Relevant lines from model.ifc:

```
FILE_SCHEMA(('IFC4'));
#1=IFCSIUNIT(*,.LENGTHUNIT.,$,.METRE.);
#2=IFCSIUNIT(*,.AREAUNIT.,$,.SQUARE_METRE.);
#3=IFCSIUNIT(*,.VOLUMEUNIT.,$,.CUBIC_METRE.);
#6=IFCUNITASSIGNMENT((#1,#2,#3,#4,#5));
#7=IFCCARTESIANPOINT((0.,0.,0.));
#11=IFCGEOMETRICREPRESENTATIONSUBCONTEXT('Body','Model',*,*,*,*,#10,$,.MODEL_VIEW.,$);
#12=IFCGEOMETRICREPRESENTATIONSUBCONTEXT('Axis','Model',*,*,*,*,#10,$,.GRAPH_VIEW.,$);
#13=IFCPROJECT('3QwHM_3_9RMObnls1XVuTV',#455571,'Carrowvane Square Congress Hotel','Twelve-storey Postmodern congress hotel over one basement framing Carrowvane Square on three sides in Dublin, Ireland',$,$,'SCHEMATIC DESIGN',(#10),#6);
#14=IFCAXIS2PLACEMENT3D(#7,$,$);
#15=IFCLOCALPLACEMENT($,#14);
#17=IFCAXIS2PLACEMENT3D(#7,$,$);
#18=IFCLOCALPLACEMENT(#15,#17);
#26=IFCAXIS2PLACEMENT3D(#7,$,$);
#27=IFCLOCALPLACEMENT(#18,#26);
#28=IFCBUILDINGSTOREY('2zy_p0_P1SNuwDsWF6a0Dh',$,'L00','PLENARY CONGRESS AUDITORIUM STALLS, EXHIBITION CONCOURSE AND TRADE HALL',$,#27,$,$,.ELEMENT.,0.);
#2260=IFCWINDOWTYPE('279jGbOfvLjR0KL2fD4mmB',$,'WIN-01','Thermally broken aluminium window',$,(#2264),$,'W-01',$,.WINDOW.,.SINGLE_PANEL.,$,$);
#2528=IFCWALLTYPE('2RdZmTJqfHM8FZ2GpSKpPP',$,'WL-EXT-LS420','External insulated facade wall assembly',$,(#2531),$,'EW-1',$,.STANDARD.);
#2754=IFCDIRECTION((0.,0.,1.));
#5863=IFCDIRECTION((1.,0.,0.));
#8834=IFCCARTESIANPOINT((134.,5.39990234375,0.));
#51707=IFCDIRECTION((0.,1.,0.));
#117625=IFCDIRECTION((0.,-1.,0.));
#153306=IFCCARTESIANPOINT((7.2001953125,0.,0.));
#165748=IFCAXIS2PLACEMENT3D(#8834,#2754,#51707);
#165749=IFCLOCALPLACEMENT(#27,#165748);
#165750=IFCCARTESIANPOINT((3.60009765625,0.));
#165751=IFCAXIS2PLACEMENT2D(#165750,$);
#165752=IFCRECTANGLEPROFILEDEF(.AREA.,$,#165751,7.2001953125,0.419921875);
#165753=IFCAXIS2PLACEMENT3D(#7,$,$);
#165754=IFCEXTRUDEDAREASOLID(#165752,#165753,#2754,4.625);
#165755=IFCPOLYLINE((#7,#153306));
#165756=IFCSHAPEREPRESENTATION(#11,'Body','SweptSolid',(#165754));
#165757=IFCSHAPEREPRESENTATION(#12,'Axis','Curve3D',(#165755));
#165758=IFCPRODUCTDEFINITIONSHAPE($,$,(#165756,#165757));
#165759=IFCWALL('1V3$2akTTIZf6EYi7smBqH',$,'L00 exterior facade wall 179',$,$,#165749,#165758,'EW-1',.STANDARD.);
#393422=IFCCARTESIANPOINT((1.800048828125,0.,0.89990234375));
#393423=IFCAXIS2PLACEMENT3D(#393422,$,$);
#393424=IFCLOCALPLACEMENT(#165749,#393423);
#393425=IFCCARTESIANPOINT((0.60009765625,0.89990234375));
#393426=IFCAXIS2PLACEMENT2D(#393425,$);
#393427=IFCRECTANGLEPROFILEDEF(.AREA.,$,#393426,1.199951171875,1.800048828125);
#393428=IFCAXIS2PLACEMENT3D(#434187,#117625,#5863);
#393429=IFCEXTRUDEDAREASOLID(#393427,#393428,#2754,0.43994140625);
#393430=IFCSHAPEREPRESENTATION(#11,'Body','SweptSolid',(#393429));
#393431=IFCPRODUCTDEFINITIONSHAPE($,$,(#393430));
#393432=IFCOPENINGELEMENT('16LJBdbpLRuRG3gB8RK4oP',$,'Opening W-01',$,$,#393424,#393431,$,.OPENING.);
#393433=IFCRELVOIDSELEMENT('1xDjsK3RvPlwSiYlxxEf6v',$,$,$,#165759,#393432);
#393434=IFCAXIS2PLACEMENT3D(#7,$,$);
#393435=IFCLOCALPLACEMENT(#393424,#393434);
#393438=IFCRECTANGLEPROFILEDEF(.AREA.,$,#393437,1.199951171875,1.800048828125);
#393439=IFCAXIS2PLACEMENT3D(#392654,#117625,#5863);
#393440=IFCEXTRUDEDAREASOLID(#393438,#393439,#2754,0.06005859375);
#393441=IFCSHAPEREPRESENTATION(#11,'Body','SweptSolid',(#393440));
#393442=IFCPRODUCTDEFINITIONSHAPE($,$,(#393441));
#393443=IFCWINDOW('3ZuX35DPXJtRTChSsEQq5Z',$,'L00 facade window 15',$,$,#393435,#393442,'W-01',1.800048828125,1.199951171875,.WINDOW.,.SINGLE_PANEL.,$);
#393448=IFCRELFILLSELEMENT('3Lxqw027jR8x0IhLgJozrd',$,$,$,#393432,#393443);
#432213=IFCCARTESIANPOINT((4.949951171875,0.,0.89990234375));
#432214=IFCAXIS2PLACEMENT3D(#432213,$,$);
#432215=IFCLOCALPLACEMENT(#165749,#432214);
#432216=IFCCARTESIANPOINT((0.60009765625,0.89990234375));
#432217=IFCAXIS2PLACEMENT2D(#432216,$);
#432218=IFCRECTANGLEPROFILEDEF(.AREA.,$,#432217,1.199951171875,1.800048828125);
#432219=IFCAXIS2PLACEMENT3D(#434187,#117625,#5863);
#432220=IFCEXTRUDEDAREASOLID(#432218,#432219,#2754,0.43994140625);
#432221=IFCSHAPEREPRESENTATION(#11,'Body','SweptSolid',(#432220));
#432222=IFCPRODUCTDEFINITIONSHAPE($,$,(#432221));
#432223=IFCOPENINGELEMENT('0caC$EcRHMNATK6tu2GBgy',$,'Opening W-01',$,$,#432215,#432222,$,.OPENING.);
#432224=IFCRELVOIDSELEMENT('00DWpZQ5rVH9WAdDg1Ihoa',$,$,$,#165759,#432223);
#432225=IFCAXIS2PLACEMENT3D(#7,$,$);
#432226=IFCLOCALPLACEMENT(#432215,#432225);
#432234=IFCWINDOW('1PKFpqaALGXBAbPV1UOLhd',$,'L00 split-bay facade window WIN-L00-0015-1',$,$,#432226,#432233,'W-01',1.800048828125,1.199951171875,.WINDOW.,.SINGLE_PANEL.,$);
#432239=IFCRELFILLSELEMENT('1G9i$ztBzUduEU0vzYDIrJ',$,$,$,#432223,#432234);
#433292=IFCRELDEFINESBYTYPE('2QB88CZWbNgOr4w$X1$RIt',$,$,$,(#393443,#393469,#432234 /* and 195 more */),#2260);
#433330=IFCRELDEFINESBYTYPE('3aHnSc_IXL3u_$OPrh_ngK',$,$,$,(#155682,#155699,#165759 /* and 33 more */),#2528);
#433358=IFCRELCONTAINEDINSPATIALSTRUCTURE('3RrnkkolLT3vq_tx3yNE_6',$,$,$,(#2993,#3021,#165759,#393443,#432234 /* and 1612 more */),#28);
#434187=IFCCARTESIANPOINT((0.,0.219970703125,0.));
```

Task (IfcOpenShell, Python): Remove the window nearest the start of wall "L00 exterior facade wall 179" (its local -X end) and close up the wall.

```python
import ifcopenshell
import ifcopenshell.api.feature
import ifcopenshell.api.root
import ifcopenshell.geom
import ifcopenshell.util.shape

model = ifcopenshell.open("model.ifc")
settings = ifcopenshell.geom.settings()


def volume(element):
    """Net volume in cubic metres, openings subtracted."""
    shape = ifcopenshell.geom.create_shape(settings, element)
    return ifcopenshell.util.shape.get_volume(shape.geometry)


window = model.by_guid("3ZuX35DPXJtRTChSsEQq5Z")
opening = window.FillsVoids[0].RelatingOpeningElement
wall = opening.VoidsElements[0].RelatingBuildingElement
before = volume(wall)

ifcopenshell.api.root.remove_product(model, product=window)
ifcopenshell.api.feature.remove_feature(model, feature=opening)

after = volume(wall)

print(f"wall volume {before:.3f} -> {after:.3f} m3")

model.write("model-out.ifc")
```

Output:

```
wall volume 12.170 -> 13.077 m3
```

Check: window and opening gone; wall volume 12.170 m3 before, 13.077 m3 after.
